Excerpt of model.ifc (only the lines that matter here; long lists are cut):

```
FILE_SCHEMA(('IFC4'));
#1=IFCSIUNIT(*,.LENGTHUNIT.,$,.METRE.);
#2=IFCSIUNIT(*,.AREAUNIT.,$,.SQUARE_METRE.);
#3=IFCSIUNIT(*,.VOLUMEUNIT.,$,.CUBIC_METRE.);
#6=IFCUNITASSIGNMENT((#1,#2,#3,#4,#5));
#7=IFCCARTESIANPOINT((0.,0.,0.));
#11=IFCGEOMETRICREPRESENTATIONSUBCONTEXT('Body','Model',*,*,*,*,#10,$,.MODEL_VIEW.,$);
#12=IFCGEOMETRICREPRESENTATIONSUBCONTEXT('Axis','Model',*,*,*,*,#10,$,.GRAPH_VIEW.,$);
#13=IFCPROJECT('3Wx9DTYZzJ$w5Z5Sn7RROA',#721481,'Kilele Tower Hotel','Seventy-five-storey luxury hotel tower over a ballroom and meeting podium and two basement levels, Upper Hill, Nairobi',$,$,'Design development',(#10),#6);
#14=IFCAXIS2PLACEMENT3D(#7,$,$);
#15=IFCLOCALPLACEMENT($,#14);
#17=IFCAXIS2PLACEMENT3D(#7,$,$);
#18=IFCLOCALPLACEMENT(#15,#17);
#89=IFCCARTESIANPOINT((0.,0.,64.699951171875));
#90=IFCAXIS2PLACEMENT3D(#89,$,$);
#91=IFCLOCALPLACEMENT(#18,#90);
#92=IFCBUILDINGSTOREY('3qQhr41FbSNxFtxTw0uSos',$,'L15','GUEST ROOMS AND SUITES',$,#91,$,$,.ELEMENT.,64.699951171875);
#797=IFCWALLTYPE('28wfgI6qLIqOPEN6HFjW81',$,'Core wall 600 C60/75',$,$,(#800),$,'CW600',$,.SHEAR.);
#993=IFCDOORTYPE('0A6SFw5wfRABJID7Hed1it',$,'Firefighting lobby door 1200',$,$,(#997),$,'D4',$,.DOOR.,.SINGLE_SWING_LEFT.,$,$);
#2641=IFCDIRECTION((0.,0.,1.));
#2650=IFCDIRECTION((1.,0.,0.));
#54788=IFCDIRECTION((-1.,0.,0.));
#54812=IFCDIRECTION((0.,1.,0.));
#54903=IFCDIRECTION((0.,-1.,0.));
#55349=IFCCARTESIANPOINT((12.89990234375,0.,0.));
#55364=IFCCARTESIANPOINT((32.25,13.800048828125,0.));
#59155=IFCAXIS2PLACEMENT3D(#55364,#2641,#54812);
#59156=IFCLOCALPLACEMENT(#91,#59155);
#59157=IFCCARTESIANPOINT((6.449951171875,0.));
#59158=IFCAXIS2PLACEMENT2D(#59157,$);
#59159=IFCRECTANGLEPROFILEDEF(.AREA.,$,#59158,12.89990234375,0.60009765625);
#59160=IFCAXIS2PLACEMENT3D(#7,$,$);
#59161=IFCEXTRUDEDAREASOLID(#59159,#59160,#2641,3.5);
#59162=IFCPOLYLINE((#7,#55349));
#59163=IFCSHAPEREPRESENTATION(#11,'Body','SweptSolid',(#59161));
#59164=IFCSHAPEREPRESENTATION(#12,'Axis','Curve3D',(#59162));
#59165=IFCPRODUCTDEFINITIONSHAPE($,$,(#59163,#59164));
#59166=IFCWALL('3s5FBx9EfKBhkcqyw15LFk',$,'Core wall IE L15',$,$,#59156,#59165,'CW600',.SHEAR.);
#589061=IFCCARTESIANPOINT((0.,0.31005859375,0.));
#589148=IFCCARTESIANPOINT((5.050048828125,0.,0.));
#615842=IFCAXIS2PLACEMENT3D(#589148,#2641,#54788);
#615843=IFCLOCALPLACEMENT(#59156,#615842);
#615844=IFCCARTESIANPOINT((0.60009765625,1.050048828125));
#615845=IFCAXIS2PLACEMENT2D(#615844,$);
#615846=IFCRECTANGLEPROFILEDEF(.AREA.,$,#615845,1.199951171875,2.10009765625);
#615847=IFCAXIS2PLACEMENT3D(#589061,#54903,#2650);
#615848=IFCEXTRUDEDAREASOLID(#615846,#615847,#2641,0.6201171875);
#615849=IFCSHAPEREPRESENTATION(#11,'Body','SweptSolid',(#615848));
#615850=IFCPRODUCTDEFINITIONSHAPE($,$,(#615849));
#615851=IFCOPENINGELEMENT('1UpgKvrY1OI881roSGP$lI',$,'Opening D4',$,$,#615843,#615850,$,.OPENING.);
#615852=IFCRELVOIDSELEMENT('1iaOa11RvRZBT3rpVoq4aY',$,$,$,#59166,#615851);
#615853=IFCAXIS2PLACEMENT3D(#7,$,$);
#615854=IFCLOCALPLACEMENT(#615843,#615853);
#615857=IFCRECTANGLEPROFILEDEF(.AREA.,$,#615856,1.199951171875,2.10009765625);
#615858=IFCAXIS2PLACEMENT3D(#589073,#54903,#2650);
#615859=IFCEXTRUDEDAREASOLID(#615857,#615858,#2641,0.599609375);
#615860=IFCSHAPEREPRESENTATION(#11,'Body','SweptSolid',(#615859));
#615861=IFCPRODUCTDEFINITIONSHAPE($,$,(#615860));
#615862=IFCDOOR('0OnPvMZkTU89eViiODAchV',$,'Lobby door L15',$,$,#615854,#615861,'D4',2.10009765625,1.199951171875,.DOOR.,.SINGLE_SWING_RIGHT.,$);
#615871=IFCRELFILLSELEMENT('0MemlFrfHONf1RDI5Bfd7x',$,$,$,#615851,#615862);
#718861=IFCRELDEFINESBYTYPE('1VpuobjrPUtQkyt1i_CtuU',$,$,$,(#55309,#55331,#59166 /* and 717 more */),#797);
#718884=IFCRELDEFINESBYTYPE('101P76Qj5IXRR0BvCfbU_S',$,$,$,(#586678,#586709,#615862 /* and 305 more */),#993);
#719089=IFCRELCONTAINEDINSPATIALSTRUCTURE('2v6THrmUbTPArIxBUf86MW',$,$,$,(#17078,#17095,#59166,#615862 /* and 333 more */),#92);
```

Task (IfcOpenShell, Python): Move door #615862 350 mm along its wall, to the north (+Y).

```python
import ifcopenshell
import ifcopenshell.api.geometry
import ifcopenshell.util.placement
import ifcopenshell.util.unit

model = ifcopenshell.open("model.ifc")
unit_scale = ifcopenshell.util.unit.calculate_unit_scale(model)

door = model.by_id(615862)
opening = door.FillsVoids[0].RelatingOpeningElement
wall = opening.VoidsElements[0].RelatingBuildingElement

wall_matrix = ifcopenshell.util.placement.get_local_placement(wall.ObjectPlacement)
shift = wall_matrix[:3, 0] * 0.35 / unit_scale
before = ifcopenshell.util.placement.get_local_placement(door.ObjectPlacement)[:3, 3].copy()

# The door is placed relative to its opening, so it follows when the opening moves.
matrix = ifcopenshell.util.placement.get_local_placement(opening.ObjectPlacement)
matrix[:3, 3] += shift
ifcopenshell.api.geometry.edit_object_placement(
    model, product=opening, matrix=matrix, is_si=False, should_transform_children=True
)

after = ifcopenshell.util.placement.get_local_placement(door.ObjectPlacement)[:3, 3]
print("door moved by", (after - before).round(3) + 0.0)

model.write("model-out.ifc")
```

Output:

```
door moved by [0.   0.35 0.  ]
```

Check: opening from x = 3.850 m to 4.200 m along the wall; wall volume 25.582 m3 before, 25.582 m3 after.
